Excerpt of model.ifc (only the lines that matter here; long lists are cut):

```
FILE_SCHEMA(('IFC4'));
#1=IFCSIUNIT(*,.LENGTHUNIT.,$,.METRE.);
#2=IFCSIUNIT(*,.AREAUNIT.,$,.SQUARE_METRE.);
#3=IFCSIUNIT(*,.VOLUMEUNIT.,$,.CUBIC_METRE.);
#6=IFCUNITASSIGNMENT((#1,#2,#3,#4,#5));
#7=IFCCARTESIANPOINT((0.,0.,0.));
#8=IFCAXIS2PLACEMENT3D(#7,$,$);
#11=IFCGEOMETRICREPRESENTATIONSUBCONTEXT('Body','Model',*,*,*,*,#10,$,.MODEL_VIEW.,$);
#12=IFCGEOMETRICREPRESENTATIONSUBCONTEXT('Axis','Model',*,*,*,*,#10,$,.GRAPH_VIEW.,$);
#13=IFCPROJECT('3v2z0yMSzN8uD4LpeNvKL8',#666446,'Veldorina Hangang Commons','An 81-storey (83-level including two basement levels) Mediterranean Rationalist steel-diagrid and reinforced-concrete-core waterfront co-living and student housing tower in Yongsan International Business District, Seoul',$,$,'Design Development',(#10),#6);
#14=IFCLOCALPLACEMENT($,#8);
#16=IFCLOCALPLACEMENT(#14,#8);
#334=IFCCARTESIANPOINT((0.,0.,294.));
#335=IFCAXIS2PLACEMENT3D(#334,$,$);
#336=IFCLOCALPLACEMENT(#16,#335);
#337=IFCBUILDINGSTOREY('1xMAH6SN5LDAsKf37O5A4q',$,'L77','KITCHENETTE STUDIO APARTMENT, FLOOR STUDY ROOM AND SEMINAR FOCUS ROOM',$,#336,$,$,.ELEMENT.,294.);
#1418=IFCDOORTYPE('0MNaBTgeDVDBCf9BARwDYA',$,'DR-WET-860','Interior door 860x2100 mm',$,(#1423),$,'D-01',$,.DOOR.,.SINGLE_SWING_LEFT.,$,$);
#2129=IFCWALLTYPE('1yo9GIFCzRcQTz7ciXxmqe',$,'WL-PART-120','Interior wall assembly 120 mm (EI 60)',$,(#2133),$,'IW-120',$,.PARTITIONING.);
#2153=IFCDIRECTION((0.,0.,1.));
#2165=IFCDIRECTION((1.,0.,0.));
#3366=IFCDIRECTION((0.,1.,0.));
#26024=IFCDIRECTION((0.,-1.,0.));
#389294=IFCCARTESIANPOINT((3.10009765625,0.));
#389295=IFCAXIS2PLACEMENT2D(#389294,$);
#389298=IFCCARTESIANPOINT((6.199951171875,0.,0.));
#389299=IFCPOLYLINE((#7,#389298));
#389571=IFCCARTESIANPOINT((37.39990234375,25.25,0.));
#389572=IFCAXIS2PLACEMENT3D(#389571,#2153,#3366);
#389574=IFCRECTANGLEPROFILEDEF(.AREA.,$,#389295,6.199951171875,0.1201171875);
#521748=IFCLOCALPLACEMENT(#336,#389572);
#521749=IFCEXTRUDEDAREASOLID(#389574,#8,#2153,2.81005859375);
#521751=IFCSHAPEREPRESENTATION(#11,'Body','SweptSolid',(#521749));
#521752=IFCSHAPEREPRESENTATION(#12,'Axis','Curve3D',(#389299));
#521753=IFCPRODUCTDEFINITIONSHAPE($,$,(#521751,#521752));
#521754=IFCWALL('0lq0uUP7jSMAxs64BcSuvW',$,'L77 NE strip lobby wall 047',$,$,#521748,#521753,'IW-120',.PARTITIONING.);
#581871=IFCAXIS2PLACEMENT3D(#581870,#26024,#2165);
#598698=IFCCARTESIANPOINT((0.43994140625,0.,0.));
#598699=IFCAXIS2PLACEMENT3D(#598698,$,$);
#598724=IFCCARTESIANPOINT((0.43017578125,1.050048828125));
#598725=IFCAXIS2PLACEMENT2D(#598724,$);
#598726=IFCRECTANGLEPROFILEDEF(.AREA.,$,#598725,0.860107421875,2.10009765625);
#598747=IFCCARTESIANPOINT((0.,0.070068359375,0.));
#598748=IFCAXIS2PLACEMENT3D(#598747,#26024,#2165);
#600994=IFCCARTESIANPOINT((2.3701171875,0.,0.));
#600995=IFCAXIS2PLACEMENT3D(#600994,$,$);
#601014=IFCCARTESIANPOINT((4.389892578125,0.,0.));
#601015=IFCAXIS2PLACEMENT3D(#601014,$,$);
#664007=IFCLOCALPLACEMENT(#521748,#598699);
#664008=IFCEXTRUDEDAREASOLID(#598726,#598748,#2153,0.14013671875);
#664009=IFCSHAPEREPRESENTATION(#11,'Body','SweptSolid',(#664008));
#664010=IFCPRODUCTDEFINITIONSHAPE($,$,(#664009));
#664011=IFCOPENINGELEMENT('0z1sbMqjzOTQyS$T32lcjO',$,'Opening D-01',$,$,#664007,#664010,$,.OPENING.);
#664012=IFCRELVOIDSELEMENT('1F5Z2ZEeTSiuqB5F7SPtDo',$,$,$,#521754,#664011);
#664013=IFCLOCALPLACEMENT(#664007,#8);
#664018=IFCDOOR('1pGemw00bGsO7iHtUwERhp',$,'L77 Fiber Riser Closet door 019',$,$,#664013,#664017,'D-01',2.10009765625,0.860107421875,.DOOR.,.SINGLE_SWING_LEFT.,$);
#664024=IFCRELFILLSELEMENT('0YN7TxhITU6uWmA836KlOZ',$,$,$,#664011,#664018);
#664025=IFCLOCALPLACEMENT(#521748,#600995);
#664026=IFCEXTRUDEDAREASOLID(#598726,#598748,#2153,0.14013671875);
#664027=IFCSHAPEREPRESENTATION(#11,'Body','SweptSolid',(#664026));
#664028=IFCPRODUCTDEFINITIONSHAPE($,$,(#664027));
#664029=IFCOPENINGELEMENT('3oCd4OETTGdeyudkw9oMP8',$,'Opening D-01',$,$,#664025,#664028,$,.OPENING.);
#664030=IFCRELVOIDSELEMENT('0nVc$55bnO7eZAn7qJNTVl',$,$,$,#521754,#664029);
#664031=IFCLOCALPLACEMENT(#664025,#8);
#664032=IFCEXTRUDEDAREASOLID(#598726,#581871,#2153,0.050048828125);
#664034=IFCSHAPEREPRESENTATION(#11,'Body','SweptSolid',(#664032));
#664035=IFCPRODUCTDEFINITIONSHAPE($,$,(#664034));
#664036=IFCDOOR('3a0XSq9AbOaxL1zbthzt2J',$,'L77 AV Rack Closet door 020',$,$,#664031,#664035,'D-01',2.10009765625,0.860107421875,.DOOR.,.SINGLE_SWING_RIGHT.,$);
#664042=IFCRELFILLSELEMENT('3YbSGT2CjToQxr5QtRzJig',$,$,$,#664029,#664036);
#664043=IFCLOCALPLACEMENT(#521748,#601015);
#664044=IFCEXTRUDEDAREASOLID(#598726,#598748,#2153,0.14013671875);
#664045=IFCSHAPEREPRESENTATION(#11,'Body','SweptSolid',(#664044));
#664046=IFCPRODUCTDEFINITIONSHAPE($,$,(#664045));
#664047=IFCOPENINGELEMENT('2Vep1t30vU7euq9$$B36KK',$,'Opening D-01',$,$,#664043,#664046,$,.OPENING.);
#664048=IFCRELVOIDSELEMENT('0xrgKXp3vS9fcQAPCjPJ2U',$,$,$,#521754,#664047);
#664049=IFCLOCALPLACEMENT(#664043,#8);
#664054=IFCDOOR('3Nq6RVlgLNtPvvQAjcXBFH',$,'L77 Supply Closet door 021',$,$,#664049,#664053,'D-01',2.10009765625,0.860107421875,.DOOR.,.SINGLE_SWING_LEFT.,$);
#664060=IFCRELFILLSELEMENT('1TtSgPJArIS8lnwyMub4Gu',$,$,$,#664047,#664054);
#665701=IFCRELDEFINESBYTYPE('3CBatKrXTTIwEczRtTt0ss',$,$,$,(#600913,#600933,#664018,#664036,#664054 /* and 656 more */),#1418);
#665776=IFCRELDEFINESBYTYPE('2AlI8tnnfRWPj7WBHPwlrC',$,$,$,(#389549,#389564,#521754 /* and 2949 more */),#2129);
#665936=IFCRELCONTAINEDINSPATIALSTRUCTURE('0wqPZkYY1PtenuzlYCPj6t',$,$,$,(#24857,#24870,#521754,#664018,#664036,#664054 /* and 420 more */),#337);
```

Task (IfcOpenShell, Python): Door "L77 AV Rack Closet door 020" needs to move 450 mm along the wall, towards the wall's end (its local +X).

```python
import ifcopenshell
import ifcopenshell.api.geometry
import ifcopenshell.util.placement
import ifcopenshell.util.unit

model = ifcopenshell.open("model.ifc")
unit_scale = ifcopenshell.util.unit.calculate_unit_scale(model)

door = model.by_id(664036)
opening = door.FillsVoids[0].RelatingOpeningElement
wall = opening.VoidsElements[0].RelatingBuildingElement

wall_matrix = ifcopenshell.util.placement.get_local_placement(wall.ObjectPlacement)
shift = wall_matrix[:3, 0] * 0.45 / unit_scale
before = ifcopenshell.util.placement.get_local_placement(door.ObjectPlacement)[:3, 3].copy()

# The door is placed relative to its opening, so it follows when the opening moves.
matrix = ifcopenshell.util.placement.get_local_placement(opening.ObjectPlacement)
matrix[:3, 3] += shift
ifcopenshell.api.geometry.edit_object_placement(
    model, product=opening, matrix=matrix, is_si=False, should_transform_children=True
)

after = ifcopenshell.util.placement.get_local_placement(door.ObjectPlacement)[:3, 3]
print("door moved by", (after - before).round(3) + 0.0)

model.write("model_v2.ifc")
```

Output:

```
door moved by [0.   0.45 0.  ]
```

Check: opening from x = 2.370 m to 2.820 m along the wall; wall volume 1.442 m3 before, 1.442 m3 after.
